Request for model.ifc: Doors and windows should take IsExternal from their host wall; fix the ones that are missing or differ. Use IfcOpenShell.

First a look at what the model holds.

```python
import ifcopenshell
import ifcopenshell.util.element

model = ifcopenshell.open("model.ifc")
print(model.schema)
seen = {}
for e in model.by_type("IfcDoor") + model.by_type("IfcWindow"):
    if not e.FillsVoids:
        continue
    host = e.FillsVoids[0].RelatingOpeningElement.VoidsElements[0].RelatingBuildingElement
    own = ifcopenshell.util.element.get_pset(e, f"Pset_{e.is_a()[3:].removesuffix('StandardCase')}Common", "IsExternal")
    wall = ifcopenshell.util.element.get_pset(host, "Pset_WallCommon", "IsExternal")
    seen[e.is_a(), own, wall] = seen.get((e.is_a(), own, wall), 0) + 1
for (cls, own, wall), count in sorted(seen.items(), key=str):
    print(count, cls, "IsExternal:", own, "| host wall:", wall)
```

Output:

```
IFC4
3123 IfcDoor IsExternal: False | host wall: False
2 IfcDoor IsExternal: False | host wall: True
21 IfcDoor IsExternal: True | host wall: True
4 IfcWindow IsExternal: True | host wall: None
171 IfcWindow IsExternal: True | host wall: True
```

```python
import ifcopenshell
import ifcopenshell.api.pset
import ifcopenshell.util.element

model = ifcopenshell.open("model.ifc")

count = 0
for ifc_class, pset_name in (("IfcDoor", "Pset_DoorCommon"), ("IfcWindow", "Pset_WindowCommon")):
    for e in model.by_type(ifc_class):
        if not e.FillsVoids:
            continue
        host = e.FillsVoids[0].RelatingOpeningElement.VoidsElements[0].RelatingBuildingElement
        external = ifcopenshell.util.element.get_pset(host, "Pset_WallCommon", "IsExternal")
        if external is None or ifcopenshell.util.element.get_pset(e, pset_name, "IsExternal") == external:
            continue
        pset = ifcopenshell.api.pset.add_pset(model, product=e, name=pset_name)
        ifcopenshell.api.pset.edit_pset(model, pset=pset, properties={"IsExternal": external})
        count += 1

print(count, "updated")

model.write("model_v2.ifc")
```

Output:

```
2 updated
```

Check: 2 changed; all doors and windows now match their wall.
